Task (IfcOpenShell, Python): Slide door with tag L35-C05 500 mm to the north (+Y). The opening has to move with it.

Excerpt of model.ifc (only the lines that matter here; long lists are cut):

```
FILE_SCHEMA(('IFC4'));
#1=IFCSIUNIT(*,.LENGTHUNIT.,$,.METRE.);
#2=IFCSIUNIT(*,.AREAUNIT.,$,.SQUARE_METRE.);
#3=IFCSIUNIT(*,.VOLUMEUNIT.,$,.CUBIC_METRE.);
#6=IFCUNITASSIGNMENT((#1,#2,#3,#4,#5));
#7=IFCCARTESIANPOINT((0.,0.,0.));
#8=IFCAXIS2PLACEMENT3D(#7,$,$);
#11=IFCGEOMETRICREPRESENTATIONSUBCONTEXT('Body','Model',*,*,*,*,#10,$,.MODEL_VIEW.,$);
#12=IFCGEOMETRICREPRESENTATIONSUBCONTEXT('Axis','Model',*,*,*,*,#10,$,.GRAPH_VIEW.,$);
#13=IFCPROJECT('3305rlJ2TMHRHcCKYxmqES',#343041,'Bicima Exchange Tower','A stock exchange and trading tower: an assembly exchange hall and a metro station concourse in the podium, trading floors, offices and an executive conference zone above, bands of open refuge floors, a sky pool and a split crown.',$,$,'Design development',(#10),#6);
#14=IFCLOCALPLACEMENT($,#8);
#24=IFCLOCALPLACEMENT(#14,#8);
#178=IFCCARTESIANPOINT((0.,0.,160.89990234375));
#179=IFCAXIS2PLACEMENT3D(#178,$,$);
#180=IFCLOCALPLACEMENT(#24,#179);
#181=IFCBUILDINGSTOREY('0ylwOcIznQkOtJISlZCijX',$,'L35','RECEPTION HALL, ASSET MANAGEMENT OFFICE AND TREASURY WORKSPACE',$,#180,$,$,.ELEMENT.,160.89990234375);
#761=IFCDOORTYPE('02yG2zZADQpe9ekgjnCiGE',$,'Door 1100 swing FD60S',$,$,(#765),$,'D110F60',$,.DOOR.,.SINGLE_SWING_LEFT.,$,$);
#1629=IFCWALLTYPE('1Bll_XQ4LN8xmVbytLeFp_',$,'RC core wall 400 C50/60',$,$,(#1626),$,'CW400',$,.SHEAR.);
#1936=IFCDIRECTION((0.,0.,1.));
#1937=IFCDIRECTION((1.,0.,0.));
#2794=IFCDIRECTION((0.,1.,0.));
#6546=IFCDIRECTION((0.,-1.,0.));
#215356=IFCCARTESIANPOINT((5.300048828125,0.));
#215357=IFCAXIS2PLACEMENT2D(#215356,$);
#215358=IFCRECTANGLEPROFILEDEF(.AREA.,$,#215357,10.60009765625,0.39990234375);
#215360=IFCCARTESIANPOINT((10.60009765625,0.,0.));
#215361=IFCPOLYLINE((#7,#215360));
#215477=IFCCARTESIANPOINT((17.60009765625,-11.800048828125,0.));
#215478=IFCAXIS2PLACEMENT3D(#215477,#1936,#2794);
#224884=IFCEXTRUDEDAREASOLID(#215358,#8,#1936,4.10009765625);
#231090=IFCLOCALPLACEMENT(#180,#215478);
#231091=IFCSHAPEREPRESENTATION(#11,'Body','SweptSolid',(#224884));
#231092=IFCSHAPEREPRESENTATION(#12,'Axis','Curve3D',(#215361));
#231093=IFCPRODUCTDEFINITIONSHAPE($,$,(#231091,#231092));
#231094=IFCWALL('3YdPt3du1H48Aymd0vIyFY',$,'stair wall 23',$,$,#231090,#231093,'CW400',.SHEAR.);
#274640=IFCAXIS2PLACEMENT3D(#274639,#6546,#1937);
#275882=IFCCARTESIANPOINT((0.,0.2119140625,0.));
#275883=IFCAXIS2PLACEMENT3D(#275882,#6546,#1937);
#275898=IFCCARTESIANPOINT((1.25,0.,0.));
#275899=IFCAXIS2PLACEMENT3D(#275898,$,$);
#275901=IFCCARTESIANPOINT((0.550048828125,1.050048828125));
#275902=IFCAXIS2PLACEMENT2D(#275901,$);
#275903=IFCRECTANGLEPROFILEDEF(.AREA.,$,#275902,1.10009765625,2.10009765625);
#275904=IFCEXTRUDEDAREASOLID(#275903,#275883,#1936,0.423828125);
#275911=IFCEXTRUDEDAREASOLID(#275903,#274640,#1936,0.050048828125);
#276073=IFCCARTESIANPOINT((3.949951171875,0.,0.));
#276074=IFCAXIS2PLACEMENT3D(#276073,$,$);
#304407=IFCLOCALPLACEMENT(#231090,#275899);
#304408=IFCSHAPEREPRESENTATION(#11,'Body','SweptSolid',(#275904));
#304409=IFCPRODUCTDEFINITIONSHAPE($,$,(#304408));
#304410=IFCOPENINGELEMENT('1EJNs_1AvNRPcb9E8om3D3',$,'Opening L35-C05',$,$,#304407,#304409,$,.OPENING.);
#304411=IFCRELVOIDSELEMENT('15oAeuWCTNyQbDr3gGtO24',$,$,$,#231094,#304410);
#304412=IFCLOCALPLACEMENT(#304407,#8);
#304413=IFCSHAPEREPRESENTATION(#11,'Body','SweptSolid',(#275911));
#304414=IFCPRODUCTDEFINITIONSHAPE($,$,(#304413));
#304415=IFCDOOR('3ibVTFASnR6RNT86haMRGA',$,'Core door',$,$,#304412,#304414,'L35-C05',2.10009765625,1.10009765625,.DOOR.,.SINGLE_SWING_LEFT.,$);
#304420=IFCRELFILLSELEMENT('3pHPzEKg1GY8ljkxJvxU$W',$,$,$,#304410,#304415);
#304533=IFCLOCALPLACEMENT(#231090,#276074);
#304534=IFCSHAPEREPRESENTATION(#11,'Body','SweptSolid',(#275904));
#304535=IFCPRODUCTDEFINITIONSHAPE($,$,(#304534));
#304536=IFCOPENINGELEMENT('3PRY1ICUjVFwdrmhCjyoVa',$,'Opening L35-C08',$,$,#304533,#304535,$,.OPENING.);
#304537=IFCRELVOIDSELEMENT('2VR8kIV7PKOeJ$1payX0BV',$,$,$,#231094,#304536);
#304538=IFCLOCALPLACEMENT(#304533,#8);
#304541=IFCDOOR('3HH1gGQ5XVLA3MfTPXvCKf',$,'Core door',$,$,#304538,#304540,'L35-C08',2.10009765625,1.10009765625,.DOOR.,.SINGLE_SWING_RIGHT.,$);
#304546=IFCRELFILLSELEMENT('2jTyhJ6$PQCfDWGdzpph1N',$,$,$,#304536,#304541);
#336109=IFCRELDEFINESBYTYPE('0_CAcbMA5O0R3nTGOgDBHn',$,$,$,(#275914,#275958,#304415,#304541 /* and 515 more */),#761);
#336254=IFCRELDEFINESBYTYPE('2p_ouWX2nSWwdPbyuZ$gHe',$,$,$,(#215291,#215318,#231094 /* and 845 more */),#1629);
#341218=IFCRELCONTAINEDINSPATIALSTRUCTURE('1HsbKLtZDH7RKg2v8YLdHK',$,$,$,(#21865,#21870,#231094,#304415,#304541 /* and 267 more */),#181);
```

```python
import ifcopenshell
import ifcopenshell.api.geometry
import ifcopenshell.util.placement
import ifcopenshell.util.unit

model = ifcopenshell.open("model.ifc")
unit_scale = ifcopenshell.util.unit.calculate_unit_scale(model)

door = model.by_id(304415)
opening = door.FillsVoids[0].RelatingOpeningElement
wall = opening.VoidsElements[0].RelatingBuildingElement

wall_matrix = ifcopenshell.util.placement.get_local_placement(wall.ObjectPlacement)
shift = wall_matrix[:3, 0] * 0.5 / unit_scale
before = ifcopenshell.util.placement.get_local_placement(door.ObjectPlacement)[:3, 3].copy()

# The door is placed relative to its opening, so it follows when the opening moves.
matrix = ifcopenshell.util.placement.get_local_placement(opening.ObjectPlacement)
matrix[:3, 3] += shift
ifcopenshell.api.geometry.edit_object_placement(
    model, product=opening, matrix=matrix, is_si=False, should_transform_children=True
)

after = ifcopenshell.util.placement.get_local_placement(door.ObjectPlacement)[:3, 3]
print("door moved by", (after - before).round(3) + 0.0)

model.write("model_edited.ifc")
```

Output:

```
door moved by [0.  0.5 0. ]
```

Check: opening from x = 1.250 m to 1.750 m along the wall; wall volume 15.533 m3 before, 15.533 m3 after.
